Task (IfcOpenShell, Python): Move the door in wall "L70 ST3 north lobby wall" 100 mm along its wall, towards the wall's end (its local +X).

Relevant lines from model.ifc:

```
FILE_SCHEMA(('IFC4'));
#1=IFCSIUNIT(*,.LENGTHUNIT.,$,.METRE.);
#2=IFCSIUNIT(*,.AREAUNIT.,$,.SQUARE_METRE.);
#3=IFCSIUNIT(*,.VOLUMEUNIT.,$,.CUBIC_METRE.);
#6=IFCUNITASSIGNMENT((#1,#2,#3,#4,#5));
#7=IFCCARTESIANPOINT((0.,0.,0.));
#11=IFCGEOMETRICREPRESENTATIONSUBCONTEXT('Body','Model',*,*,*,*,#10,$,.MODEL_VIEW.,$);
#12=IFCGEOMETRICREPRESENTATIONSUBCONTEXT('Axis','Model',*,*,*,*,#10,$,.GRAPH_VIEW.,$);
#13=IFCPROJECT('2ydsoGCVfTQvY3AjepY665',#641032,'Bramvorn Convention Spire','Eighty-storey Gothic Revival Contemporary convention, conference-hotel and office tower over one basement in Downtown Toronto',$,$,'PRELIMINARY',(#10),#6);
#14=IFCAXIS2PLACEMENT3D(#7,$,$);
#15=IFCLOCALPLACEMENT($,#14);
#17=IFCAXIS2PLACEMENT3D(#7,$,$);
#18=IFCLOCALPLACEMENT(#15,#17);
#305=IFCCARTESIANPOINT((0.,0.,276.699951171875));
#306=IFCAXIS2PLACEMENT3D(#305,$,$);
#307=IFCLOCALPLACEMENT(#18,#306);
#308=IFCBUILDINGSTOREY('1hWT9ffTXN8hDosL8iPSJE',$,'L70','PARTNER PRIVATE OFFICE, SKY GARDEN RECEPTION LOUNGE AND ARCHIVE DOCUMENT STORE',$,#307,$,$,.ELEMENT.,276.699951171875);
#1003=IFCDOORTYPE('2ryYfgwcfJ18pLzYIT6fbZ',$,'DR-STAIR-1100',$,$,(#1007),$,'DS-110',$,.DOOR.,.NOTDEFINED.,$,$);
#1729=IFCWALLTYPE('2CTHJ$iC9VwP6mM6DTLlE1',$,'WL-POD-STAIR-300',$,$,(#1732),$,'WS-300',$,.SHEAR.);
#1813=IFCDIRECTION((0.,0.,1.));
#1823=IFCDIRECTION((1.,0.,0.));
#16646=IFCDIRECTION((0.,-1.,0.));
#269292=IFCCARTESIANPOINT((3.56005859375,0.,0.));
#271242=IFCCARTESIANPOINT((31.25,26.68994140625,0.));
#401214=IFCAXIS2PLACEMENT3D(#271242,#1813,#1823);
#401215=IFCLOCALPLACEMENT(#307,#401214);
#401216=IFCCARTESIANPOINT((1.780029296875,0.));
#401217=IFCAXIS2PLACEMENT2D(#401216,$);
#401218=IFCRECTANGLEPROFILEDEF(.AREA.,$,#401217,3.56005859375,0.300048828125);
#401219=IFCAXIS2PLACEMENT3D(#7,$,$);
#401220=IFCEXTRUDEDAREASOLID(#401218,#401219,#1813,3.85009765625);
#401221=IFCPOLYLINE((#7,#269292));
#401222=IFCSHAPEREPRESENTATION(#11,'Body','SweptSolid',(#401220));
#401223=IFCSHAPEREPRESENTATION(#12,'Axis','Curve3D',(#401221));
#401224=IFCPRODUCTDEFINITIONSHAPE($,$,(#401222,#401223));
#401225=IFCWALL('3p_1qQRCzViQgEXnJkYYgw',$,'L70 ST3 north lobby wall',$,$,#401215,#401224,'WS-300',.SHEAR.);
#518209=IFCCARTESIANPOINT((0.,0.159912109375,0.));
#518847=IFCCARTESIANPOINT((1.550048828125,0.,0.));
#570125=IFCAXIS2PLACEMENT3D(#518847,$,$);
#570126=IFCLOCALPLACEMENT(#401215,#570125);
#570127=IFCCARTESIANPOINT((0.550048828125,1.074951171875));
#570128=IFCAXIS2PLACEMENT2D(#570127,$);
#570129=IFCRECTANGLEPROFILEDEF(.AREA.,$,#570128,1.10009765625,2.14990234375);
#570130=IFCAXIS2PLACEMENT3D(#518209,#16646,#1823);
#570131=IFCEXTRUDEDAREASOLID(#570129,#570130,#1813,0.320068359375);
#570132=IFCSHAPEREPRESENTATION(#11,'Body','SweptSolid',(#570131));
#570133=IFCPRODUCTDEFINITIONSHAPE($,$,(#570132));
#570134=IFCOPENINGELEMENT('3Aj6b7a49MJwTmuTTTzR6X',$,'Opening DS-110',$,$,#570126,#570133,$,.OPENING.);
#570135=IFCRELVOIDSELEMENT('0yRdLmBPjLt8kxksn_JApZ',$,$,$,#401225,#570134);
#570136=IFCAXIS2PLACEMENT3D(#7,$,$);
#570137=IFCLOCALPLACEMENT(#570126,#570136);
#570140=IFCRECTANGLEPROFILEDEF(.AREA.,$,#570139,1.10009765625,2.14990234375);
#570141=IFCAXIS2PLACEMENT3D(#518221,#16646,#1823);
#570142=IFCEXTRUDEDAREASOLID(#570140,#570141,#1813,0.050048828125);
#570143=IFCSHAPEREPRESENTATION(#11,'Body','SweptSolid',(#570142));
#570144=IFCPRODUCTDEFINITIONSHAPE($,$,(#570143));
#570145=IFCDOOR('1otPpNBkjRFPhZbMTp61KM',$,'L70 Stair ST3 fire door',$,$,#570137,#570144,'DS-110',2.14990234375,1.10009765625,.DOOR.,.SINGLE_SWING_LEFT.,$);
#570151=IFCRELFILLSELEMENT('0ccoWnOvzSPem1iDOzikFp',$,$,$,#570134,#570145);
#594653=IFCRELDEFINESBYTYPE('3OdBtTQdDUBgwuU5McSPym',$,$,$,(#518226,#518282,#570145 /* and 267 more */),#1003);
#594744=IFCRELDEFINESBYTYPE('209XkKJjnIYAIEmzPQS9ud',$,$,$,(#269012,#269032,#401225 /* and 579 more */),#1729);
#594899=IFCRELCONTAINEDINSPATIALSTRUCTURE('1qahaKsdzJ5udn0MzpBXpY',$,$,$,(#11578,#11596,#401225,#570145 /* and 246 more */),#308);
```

```python
import ifcopenshell
import ifcopenshell.api.geometry
import ifcopenshell.util.placement

model = ifcopenshell.open("model.ifc")

door = model.by_id(570145)
opening = door.FillsVoids[0].RelatingOpeningElement
wall = opening.VoidsElements[0].RelatingBuildingElement

wall_matrix = ifcopenshell.util.placement.get_local_placement(wall.ObjectPlacement)
shift = wall_matrix[:3, 0] * 0.1
before = ifcopenshell.util.placement.get_local_placement(door.ObjectPlacement)[:3, 3].copy()

# The door is placed relative to its opening, so it follows when the opening moves.
matrix = ifcopenshell.util.placement.get_local_placement(opening.ObjectPlacement)
matrix[:3, 3] += shift
ifcopenshell.api.geometry.edit_object_placement(
    model, product=opening, matrix=matrix, is_si=False, should_transform_children=True
)

after = ifcopenshell.util.placement.get_local_placement(door.ObjectPlacement)[:3, 3]
print("door moved by", (after - before).round(3) + 0.0)

model.write("model_edited.ifc")
```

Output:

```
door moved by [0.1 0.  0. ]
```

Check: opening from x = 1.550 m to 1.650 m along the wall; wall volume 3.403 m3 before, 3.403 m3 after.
